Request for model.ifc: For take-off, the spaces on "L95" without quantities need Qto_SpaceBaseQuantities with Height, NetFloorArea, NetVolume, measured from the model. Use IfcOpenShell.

First a look at what the model holds.

```python
import ifcopenshell
import ifcopenshell.util.element
import ifcopenshell.util.unit

model = ifcopenshell.open("model.ifc")
print(model.schema)
for unit_type in ("LENGTHUNIT", "AREAUNIT", "VOLUMEUNIT"):
    print(unit_type, ifcopenshell.util.unit.calculate_unit_scale(model, unit_type))
storey = next(s for s in model.by_type("IfcBuildingStorey") if s.Name == "L95")
spaces = [e for e in ifcopenshell.util.element.get_decomposition(storey) if e.is_a("IfcSpace")]
for e in sorted(spaces, key=lambda e: e.id()):
    print(e.id(), e.is_a(), e.Name, list(ifcopenshell.util.element.get_psets(e, qtos_only=True)), sep=" | ")
```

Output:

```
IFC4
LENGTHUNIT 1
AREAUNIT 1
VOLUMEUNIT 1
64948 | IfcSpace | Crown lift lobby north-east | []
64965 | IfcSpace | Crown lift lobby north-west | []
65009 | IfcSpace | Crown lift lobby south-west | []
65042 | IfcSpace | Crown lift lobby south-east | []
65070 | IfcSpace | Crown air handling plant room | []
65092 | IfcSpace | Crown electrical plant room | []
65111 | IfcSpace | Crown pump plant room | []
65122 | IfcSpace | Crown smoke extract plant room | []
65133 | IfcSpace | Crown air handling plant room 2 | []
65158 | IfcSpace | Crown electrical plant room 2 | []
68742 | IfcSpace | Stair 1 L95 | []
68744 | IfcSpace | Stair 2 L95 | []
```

```python
import ifcopenshell
import ifcopenshell.api.pset
import ifcopenshell.geom
import ifcopenshell.util.element
import ifcopenshell.util.shape
import ifcopenshell.util.unit

model = ifcopenshell.open("model.ifc")
unit_scale = ifcopenshell.util.unit.calculate_unit_scale(model)
area_scale = ifcopenshell.util.unit.calculate_unit_scale(model, "AREAUNIT")
volume_scale = ifcopenshell.util.unit.calculate_unit_scale(model, "VOLUMEUNIT")
settings = ifcopenshell.geom.settings()

storey = next(s for s in model.by_type("IfcBuildingStorey") if s.Name == "L95")
spaces = [e for e in ifcopenshell.util.element.get_decomposition(storey) if e.is_a("IfcSpace")]

for e in sorted(spaces, key=lambda e: e.id()):
    if ifcopenshell.util.element.get_psets(e, qtos_only=True, should_inherit=False):
        continue
    # Geometry comes back in metres, in the element's own axes.
    shape = ifcopenshell.geom.create_shape(settings, e)
    values = {
        "Height": ifcopenshell.util.shape.get_z(shape.geometry) / unit_scale,
        "NetFloorArea": ifcopenshell.util.shape.get_footprint_area(shape.geometry) / area_scale,
        "NetVolume": ifcopenshell.util.shape.get_volume(shape.geometry) / volume_scale,
    }
    qto = ifcopenshell.api.pset.add_qto(model, product=e, name="Qto_SpaceBaseQuantities")
    ifcopenshell.api.pset.edit_qto(model, qto=qto, properties=values)
    print(e.id(), {k: round(v, 3) for k, v in values.items()})

model.write("model_rev.ifc")
```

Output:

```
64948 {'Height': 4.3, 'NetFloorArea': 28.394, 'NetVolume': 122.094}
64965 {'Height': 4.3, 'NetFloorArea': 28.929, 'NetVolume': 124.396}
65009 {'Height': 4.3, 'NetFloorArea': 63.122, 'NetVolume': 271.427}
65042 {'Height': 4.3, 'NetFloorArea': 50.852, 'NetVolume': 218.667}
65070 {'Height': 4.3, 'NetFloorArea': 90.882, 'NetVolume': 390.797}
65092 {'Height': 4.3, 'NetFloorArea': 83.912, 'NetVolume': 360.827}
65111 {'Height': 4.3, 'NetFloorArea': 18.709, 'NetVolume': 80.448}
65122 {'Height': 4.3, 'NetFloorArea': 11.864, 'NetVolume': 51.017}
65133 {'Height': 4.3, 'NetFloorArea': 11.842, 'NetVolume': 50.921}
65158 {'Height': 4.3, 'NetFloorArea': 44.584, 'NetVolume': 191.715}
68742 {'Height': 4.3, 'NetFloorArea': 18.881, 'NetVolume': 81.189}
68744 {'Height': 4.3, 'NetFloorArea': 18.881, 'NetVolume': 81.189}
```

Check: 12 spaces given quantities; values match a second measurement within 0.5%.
